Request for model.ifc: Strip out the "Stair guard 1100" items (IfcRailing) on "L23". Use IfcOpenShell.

First a look at what the model holds.

```python
import ifcopenshell
import ifcopenshell.util.element

model = ifcopenshell.open("model.ifc")
print(model.schema)
storey = next(s for s in model.by_type("IfcBuildingStorey") if s.Name == "L23")
railings = [e for e in ifcopenshell.util.element.get_decomposition(storey) if e.is_a("IfcRailing")]
seen = {}
for e in railings:
    element_type = ifcopenshell.util.element.get_type(e)
    name = element_type.Name if element_type not in (None, e) else None
    seen[name] = seen.get(name, 0) + 1
for name, count in sorted(seen.items(), key=str):
    print(count, "x", name)
```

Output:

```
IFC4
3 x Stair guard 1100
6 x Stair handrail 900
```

```python
import ifcopenshell
import ifcopenshell.api.root
import ifcopenshell.util.element

model = ifcopenshell.open("model.ifc")

storey = next(s for s in model.by_type("IfcBuildingStorey") if s.Name == "L23")
railings = [e for e in ifcopenshell.util.element.get_decomposition(storey) if e.is_a("IfcRailing")]
targets = [e for e in railings if (t := ifcopenshell.util.element.get_type(e)) not in (None, e) and t.Name == "Stair guard 1100"]

for e in targets:
    ifcopenshell.api.root.remove_product(model, product=e)
print(len(targets), "removed")

model.write("model_rev.ifc")
```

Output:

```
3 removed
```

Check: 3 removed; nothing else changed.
